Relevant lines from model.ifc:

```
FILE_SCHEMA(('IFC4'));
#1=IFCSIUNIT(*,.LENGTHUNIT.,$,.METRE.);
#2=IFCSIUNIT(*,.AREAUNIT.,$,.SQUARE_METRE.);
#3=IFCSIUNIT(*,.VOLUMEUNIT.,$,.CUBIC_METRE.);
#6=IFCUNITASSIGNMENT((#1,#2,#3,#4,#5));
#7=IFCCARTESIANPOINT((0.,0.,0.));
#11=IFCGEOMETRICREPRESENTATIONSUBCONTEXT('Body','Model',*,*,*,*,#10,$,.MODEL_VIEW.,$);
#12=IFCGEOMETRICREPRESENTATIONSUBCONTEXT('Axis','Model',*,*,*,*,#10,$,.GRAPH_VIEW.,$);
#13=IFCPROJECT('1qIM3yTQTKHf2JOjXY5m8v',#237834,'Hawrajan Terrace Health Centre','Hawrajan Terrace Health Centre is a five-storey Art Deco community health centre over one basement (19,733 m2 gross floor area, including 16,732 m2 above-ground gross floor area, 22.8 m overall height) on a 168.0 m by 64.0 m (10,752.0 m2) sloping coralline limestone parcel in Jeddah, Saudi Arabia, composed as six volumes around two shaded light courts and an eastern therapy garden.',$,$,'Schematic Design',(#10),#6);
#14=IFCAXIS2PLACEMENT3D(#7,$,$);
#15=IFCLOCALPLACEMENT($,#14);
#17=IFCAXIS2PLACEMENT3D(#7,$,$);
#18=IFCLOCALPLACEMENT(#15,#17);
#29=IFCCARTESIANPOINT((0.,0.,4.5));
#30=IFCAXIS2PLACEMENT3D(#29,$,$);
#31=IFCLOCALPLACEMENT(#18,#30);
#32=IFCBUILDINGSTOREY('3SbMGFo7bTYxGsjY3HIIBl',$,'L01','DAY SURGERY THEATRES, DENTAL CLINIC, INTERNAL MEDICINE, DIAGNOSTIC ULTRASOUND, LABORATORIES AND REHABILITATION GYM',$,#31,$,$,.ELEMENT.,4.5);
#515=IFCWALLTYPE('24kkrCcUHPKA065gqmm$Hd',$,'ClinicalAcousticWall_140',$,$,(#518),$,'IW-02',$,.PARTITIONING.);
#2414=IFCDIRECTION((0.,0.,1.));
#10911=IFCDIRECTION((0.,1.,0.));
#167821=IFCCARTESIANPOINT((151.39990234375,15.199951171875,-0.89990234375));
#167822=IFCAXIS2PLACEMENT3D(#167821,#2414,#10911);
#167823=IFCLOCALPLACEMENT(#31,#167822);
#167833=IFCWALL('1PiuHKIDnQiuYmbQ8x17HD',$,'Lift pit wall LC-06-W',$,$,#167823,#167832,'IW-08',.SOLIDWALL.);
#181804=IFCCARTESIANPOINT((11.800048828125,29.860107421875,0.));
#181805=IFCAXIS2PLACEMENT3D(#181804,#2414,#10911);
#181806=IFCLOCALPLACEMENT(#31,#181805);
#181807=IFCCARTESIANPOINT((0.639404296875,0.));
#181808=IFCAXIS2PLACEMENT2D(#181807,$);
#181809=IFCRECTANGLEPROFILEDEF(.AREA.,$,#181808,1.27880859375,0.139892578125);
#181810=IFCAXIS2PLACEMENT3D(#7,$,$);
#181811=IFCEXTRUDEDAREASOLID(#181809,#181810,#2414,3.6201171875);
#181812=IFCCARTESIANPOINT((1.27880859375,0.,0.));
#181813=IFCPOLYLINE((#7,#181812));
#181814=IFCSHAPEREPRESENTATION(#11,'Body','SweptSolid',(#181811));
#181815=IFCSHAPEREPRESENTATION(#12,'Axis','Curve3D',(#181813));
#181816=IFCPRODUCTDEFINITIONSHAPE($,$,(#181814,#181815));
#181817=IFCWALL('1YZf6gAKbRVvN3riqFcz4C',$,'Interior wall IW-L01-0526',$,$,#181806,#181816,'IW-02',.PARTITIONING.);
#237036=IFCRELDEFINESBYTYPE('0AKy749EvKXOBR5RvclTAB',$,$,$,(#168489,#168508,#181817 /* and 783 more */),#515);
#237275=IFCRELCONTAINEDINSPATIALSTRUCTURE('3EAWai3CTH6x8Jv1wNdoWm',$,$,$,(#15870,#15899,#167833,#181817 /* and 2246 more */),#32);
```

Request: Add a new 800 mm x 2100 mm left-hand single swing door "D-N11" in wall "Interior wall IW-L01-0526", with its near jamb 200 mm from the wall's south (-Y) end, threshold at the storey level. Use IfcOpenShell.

```python
import numpy as np
import ifcopenshell
import ifcopenshell.api.feature
import ifcopenshell.api.geometry
import ifcopenshell.api.root
import ifcopenshell.api.spatial
import ifcopenshell.geom
import ifcopenshell.util.element
import ifcopenshell.util.placement
import ifcopenshell.util.representation
import ifcopenshell.util.shape
import ifcopenshell.util.unit

model = ifcopenshell.open("model.ifc")
unit_scale = ifcopenshell.util.unit.calculate_unit_scale(model)
settings = ifcopenshell.geom.settings()


def volume(element):
    """Net volume in cubic metres, openings subtracted."""
    shape = ifcopenshell.geom.create_shape(settings, element)
    return ifcopenshell.util.shape.get_volume(shape.geometry)


wall = model.by_id(181817)
storey = ifcopenshell.util.element.get_container(wall, ifc_class="IfcBuildingStorey")
context = ifcopenshell.util.representation.get_context(model, "Model", "Body", "MODEL_VIEW")
before = volume(wall)

width, height, from_end, sill = 0.8, 2.1, 0.2, 0.0  # metres

# The wall runs along its own X axis, and the end named is its -X end.
wall_shape = ifcopenshell.geom.create_shape(settings, wall)
x, y, z = ifcopenshell.util.shape.get_vertices(wall_shape.geometry).T
start = x.min() + from_end
face, thickness = float(y.min()), float(y.max() - y.min())
wall_matrix = ifcopenshell.util.placement.get_local_placement(wall.ObjectPlacement)
level = ifcopenshell.util.placement.get_local_placement(storey.ObjectPlacement)[2, 3]


def in_wall(x, y):
    """Placement at x, y metres in the wall's axes, at sill height."""
    matrix = wall_matrix.copy()
    matrix[:, 3] = wall_matrix @ np.array([x / unit_scale, y / unit_scale, 0.0, 1.0])
    matrix[2, 3] = level + sill / unit_scale
    return matrix


# Opening: a box that overshoots both wall faces by 50 mm.
opening = ifcopenshell.api.root.create_entity(model, ifc_class="IfcOpeningElement", predefined_type="OPENING")
box = ifcopenshell.api.geometry.add_wall_representation(
    model, context=context, length=width, height=height, thickness=thickness + 0.1
)
ifcopenshell.api.geometry.assign_representation(model, product=opening, representation=box)
ifcopenshell.api.geometry.edit_object_placement(model, product=opening, matrix=in_wall(start, face - 0.05), is_si=False)
ifcopenshell.api.feature.add_feature(model, feature=opening, element=wall)

door = ifcopenshell.api.root.create_entity(model, ifc_class="IfcDoor", name="D-N11", predefined_type="DOOR")
door.OverallWidth, door.OverallHeight = width / unit_scale, height / unit_scale
door.OperationType = "SINGLE_SWING_LEFT"
body = ifcopenshell.api.geometry.add_door_representation(
    model,
    context=context,
    overall_width=door.OverallWidth,
    overall_height=door.OverallHeight,
    operation_type="SINGLE_SWING_LEFT",
    lining_properties={"LiningDepth": thickness / unit_scale, "ThresholdDepth": thickness / unit_scale},
)
ifcopenshell.api.geometry.assign_representation(model, product=door, representation=body)
ifcopenshell.api.spatial.assign_container(model, products=[door], relating_structure=storey)
ifcopenshell.api.feature.add_filling(model, opening=opening, element=door)

# The lining spans the wall, so the door starts at the wall face.
ifcopenshell.api.geometry.edit_object_placement(model, product=door, matrix=in_wall(start, face), is_si=False)

after = volume(wall)

print(f"wall volume {before:.3f} -> {after:.3f} m3")

model.write("model_v2.ifc")
```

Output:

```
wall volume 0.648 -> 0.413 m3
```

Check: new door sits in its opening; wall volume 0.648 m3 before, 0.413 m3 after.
